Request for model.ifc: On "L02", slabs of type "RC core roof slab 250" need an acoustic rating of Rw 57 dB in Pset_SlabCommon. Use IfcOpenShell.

First a look at what the model holds.

```python
import ifcopenshell
import ifcopenshell.util.element

model = ifcopenshell.open("model.ifc")
print(model.schema)
storey = next(s for s in model.by_type("IfcBuildingStorey") if s.Name == "L02")
slabs = [e for e in ifcopenshell.util.element.get_decomposition(storey) if e.is_a("IfcSlab")]
seen = {}
for e in slabs:
    element_type = ifcopenshell.util.element.get_type(e)
    key = (element_type.Name if element_type != e and element_type else None, ifcopenshell.util.element.get_pset(e, "Pset_SlabCommon", "AcousticRating"))
    seen[key] = seen.get(key, 0) + 1
for (name, value), count in sorted(seen.items(), key=str):
    print(count, "x", name, "|", value)
```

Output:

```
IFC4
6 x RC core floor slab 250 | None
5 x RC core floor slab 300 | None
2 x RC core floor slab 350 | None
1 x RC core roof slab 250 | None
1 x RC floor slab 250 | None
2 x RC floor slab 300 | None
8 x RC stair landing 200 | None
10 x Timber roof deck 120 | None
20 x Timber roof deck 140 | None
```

```python
import ifcopenshell
import ifcopenshell.api.pset
import ifcopenshell.util.element

model = ifcopenshell.open("model.ifc")

storey = next(s for s in model.by_type("IfcBuildingStorey") if s.Name == "L02")
slabs = [e for e in ifcopenshell.util.element.get_decomposition(storey) if e.is_a("IfcSlab")]

count = 0
for e in slabs:
    element_type = ifcopenshell.util.element.get_type(e)
    if element_type in (None, e) or element_type.Name != "RC core roof slab 250":
        continue
    # add_pset returns the element's existing set when there is one.
    pset = ifcopenshell.api.pset.add_pset(model, product=e, name="Pset_SlabCommon")
    ifcopenshell.api.pset.edit_pset(model, pset=pset, properties={"AcousticRating": "Rw 57 dB"})
    count += 1

print(count, "slabs updated")

model.write("model_updated.ifc")
```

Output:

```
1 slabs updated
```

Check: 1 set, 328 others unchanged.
